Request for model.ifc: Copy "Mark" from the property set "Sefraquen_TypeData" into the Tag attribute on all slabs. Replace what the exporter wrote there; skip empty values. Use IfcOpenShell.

First a look at what the model holds.

```python
import ifcopenshell
import ifcopenshell.util.element

model = ifcopenshell.open("model.ifc")
print(model.schema)
slabs = model.by_type("IfcSlab")
print(len(slabs), "slabs")
for e in slabs[:8]:
    source = ifcopenshell.util.element.get_pset(e, "Sefraquen_TypeData", "Mark")
    target = e.Tag
    print(e.id(), repr(source), repr(target), sep=" | ")
```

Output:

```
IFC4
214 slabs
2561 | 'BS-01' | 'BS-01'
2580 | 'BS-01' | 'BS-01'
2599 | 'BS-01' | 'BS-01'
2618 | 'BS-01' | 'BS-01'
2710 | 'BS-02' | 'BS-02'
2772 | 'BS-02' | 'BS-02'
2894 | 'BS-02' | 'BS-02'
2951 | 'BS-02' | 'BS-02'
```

```python
import ifcopenshell
import ifcopenshell.util.element

model = ifcopenshell.open("model.ifc")

count = 0
for e in model.by_type("IfcSlab"):
    value = ifcopenshell.util.element.get_pset(e, "Sefraquen_TypeData", "Mark")
    current = e.Tag
    if not value or not value.strip() or current == value:
        continue
    e.Tag = value
    count += 1

print(count, "slabs updated")

model.write("model-out.ifc")
```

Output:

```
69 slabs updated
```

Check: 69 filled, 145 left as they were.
